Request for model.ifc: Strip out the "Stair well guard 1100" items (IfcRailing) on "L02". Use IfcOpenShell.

First a look at what the model holds.

```python
import ifcopenshell
import ifcopenshell.util.element

model = ifcopenshell.open("model.ifc")
print(model.schema)
storey = next(s for s in model.by_type("IfcBuildingStorey") if s.Name == "L02")
railings = [e for e in ifcopenshell.util.element.get_decomposition(storey) if e.is_a("IfcRailing")]
seen = {}
for e in railings:
    element_type = ifcopenshell.util.element.get_type(e)
    name = element_type.Name if element_type not in (None, e) else None
    seen[name] = seen.get(name, 0) + 1
for name, count in sorted(seen.items(), key=str):
    print(count, "x", name)
```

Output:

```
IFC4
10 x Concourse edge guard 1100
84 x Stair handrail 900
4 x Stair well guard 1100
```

```python
import ifcopenshell
import ifcopenshell.api.root
import ifcopenshell.util.element

model = ifcopenshell.open("model.ifc")

storey = next(s for s in model.by_type("IfcBuildingStorey") if s.Name == "L02")
railings = [e for e in ifcopenshell.util.element.get_decomposition(storey) if e.is_a("IfcRailing")]
targets = [e for e in railings if (t := ifcopenshell.util.element.get_type(e)) not in (None, e) and t.Name == "Stair well guard 1100"]

for e in targets:
    ifcopenshell.api.root.remove_product(model, product=e)
print(len(targets), "removed")

model.write("model_updated.ifc")
```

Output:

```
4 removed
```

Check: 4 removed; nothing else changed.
